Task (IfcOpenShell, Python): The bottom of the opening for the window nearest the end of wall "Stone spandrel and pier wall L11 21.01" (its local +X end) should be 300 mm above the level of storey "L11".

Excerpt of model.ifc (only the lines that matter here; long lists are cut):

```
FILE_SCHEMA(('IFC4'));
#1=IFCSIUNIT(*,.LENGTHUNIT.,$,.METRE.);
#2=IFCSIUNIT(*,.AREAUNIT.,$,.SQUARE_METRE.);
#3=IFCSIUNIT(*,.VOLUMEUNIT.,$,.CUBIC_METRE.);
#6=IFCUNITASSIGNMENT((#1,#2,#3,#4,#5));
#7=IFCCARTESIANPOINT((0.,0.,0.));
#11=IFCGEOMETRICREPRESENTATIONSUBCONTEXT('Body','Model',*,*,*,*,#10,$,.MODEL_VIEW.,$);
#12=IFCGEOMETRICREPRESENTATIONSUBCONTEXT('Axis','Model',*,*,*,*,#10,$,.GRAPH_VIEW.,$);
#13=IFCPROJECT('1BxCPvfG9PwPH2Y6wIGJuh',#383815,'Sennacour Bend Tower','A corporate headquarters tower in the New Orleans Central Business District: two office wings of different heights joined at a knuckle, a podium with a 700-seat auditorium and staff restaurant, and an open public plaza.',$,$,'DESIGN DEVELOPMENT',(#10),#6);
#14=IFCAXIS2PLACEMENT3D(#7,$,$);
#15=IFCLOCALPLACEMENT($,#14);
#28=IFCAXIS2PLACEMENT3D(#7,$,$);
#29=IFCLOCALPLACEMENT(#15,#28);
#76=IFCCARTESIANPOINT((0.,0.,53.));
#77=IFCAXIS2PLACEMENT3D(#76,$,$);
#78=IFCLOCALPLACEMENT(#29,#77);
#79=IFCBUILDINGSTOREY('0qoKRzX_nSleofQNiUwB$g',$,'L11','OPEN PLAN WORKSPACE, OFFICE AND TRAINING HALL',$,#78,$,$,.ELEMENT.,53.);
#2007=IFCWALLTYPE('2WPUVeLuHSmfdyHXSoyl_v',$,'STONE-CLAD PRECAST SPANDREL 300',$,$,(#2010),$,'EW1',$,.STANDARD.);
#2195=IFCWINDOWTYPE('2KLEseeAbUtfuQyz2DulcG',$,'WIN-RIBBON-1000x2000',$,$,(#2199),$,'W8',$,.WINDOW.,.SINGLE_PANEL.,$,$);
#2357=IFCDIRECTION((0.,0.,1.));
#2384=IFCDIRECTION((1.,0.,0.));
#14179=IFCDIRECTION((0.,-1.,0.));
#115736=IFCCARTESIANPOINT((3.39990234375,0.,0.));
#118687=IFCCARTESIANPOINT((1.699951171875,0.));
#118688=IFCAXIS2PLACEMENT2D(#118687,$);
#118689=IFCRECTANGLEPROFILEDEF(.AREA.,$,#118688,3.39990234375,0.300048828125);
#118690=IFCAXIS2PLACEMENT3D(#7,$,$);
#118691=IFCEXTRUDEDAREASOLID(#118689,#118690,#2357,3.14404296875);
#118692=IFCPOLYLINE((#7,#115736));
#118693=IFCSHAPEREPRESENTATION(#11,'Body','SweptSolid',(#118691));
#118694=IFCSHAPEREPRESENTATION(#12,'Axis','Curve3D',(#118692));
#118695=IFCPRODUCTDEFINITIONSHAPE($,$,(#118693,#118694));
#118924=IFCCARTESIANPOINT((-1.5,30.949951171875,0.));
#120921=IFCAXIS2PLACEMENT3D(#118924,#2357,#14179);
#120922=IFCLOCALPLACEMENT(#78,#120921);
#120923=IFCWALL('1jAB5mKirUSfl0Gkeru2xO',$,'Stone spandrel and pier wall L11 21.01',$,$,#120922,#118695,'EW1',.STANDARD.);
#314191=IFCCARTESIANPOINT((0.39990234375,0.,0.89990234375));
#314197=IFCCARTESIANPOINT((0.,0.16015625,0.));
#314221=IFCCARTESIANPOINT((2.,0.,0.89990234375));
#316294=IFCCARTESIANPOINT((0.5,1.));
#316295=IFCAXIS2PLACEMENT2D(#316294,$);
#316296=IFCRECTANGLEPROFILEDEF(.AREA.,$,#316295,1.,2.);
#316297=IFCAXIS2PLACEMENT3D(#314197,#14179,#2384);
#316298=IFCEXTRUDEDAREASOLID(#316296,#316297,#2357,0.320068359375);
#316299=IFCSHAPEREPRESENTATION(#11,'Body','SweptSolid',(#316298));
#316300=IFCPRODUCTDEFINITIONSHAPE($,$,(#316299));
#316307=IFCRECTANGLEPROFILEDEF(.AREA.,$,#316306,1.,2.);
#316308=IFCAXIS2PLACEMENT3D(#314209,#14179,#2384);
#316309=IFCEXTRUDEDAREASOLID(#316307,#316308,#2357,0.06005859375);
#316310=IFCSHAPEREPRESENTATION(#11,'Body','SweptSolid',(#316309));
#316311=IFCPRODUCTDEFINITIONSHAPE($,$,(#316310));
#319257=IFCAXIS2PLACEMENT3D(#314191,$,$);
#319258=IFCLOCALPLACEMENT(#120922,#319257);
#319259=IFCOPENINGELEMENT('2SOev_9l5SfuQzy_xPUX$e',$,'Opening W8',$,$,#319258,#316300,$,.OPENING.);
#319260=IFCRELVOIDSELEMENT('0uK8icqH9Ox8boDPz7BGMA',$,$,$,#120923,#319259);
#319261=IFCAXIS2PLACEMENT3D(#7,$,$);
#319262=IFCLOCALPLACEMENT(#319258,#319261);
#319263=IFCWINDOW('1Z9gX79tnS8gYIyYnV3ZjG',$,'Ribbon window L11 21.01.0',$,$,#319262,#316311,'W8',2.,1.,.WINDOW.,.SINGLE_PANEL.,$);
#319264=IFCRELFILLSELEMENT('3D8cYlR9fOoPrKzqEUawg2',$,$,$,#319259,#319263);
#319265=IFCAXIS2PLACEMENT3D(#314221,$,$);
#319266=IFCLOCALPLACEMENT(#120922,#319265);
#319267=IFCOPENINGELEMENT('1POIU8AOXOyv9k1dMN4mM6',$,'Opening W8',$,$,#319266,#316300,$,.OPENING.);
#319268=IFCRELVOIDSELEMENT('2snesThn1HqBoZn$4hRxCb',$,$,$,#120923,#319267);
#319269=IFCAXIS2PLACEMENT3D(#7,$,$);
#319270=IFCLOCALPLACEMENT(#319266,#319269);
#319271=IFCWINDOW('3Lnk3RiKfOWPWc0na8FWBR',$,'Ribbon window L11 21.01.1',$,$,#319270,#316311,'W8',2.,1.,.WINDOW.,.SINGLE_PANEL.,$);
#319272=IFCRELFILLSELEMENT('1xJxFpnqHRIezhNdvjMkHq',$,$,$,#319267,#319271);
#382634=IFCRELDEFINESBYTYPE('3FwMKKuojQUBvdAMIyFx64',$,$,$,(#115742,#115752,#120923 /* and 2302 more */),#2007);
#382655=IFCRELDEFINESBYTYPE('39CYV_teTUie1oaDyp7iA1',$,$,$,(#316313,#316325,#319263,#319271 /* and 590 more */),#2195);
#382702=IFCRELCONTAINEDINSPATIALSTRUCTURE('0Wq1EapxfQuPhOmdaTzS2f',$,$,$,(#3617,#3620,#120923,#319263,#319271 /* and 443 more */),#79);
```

```python
import numpy as np
import ifcopenshell
import ifcopenshell.api.geometry
import ifcopenshell.geom
import ifcopenshell.util.element
import ifcopenshell.util.placement
import ifcopenshell.util.shape
import ifcopenshell.util.unit

model = ifcopenshell.open("model.ifc")
unit_scale = ifcopenshell.util.unit.calculate_unit_scale(model)

window = model.by_guid("3Lnk3RiKfOWPWc0na8FWBR")
opening = window.FillsVoids[0].RelatingOpeningElement
storey = ifcopenshell.util.element.get_container(window, ifc_class="IfcBuildingStorey")
level = ifcopenshell.util.placement.get_local_placement(storey.ObjectPlacement)[2, 3]

# The opening's origin need not be at the sill, so measure its lowest point.
shape = ifcopenshell.geom.create_shape(ifcopenshell.geom.settings(), opening)
bottom = ifcopenshell.util.shape.get_shape_bottom_elevation(shape, shape.geometry) / unit_scale
dz = level + 0.3 - bottom

shift = np.array([0.0, 0.0, dz])
# The window is placed relative to its opening, so it follows when the opening moves.
matrix = ifcopenshell.util.placement.get_local_placement(opening.ObjectPlacement)
matrix[:3, 3] += shift
ifcopenshell.api.geometry.edit_object_placement(
    model, product=opening, matrix=matrix, is_si=False, should_transform_children=True
)

print(f"moved by {dz * unit_scale:+.3f} m")

model.write("model_rev.ifc")
```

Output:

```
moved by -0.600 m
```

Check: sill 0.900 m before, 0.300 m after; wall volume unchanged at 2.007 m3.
